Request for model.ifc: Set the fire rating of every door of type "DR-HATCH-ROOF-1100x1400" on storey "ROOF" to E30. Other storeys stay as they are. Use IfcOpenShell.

First a look at what the model holds.

```python
import ifcopenshell
import ifcopenshell.util.element

model = ifcopenshell.open("model.ifc")
print(model.schema)
storey = next(s for s in model.by_type("IfcBuildingStorey") if s.Name == "ROOF")
doors = [e for e in ifcopenshell.util.element.get_decomposition(storey) if e.is_a("IfcDoor")]
seen = {}
for e in doors:
    element_type = ifcopenshell.util.element.get_type(e)
    key = (element_type.Name if element_type != e and element_type else None, ifcopenshell.util.element.get_pset(e, "Pset_DoorCommon", "FireRating"))
    seen[key] = seen.get(key, 0) + 1
for (name, value), count in sorted(seen.items(), key=str):
    print(count, "x", name, "|", value)
```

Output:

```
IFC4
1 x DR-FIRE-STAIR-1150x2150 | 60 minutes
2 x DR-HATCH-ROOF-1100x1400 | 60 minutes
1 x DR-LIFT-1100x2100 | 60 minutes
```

```python
import ifcopenshell
import ifcopenshell.api.pset
import ifcopenshell.util.element

model = ifcopenshell.open("model.ifc")

storey = next(s for s in model.by_type("IfcBuildingStorey") if s.Name == "ROOF")
doors = [e for e in ifcopenshell.util.element.get_decomposition(storey) if e.is_a("IfcDoor")]

count = 0
for e in doors:
    element_type = ifcopenshell.util.element.get_type(e)
    if element_type in (None, e) or element_type.Name != "DR-HATCH-ROOF-1100x1400":
        continue
    # add_pset returns the element's existing set when there is one.
    pset = ifcopenshell.api.pset.add_pset(model, product=e, name="Pset_DoorCommon")
    ifcopenshell.api.pset.edit_pset(model, pset=pset, properties={"FireRating": "E30"})
    count += 1

print(count, "doors updated")

model.write("model-out.ifc")
```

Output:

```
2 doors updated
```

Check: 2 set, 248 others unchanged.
